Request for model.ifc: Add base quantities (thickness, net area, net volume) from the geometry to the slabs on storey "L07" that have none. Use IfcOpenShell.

First a look at what the model holds.

```python
import ifcopenshell
import ifcopenshell.util.element
import ifcopenshell.util.unit

model = ifcopenshell.open("model.ifc")
print(model.schema)
for unit_type in ("LENGTHUNIT", "AREAUNIT", "VOLUMEUNIT"):
    print(unit_type, ifcopenshell.util.unit.calculate_unit_scale(model, unit_type))
storey = next(s for s in model.by_type("IfcBuildingStorey") if s.Name == "L07")
slabs = [e for e in ifcopenshell.util.element.get_decomposition(storey) if e.is_a("IfcSlab")]
for e in sorted(slabs, key=lambda e: e.id()):
    print(e.id(), e.is_a(), e.Name, list(ifcopenshell.util.element.get_psets(e, qtos_only=True)), sep=" | ")
```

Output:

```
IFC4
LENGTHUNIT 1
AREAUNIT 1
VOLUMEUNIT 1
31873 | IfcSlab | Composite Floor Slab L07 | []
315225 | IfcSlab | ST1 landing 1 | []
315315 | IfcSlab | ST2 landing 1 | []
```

```python
import ifcopenshell
import ifcopenshell.api.pset
import ifcopenshell.geom
import ifcopenshell.util.element
import ifcopenshell.util.shape
import ifcopenshell.util.unit

model = ifcopenshell.open("model.ifc")
unit_scale = ifcopenshell.util.unit.calculate_unit_scale(model)
area_scale = ifcopenshell.util.unit.calculate_unit_scale(model, "AREAUNIT")
volume_scale = ifcopenshell.util.unit.calculate_unit_scale(model, "VOLUMEUNIT")
settings = ifcopenshell.geom.settings()

storey = next(s for s in model.by_type("IfcBuildingStorey") if s.Name == "L07")
slabs = [e for e in ifcopenshell.util.element.get_decomposition(storey) if e.is_a("IfcSlab")]

for e in sorted(slabs, key=lambda e: e.id()):
    if ifcopenshell.util.element.get_psets(e, qtos_only=True, should_inherit=False):
        continue
    # Geometry comes back in metres, in the element's own axes.
    shape = ifcopenshell.geom.create_shape(settings, e)
    values = {
        "Width": ifcopenshell.util.shape.get_z(shape.geometry) / unit_scale,
        "NetArea": ifcopenshell.util.shape.get_footprint_area(shape.geometry) / area_scale,
        "NetVolume": ifcopenshell.util.shape.get_volume(shape.geometry) / volume_scale,
    }
    qto = ifcopenshell.api.pset.add_qto(model, product=e, name="Qto_SlabBaseQuantities")
    ifcopenshell.api.pset.edit_qto(model, qto=qto, properties=values)
    print(e.id(), {k: round(v, 3) for k, v in values.items()})

model.write("model_rev.ifc")
```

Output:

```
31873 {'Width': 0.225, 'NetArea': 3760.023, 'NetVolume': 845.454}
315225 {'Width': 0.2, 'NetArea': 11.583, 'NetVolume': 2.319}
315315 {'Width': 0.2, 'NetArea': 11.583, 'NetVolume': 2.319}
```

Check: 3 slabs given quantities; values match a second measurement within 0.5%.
